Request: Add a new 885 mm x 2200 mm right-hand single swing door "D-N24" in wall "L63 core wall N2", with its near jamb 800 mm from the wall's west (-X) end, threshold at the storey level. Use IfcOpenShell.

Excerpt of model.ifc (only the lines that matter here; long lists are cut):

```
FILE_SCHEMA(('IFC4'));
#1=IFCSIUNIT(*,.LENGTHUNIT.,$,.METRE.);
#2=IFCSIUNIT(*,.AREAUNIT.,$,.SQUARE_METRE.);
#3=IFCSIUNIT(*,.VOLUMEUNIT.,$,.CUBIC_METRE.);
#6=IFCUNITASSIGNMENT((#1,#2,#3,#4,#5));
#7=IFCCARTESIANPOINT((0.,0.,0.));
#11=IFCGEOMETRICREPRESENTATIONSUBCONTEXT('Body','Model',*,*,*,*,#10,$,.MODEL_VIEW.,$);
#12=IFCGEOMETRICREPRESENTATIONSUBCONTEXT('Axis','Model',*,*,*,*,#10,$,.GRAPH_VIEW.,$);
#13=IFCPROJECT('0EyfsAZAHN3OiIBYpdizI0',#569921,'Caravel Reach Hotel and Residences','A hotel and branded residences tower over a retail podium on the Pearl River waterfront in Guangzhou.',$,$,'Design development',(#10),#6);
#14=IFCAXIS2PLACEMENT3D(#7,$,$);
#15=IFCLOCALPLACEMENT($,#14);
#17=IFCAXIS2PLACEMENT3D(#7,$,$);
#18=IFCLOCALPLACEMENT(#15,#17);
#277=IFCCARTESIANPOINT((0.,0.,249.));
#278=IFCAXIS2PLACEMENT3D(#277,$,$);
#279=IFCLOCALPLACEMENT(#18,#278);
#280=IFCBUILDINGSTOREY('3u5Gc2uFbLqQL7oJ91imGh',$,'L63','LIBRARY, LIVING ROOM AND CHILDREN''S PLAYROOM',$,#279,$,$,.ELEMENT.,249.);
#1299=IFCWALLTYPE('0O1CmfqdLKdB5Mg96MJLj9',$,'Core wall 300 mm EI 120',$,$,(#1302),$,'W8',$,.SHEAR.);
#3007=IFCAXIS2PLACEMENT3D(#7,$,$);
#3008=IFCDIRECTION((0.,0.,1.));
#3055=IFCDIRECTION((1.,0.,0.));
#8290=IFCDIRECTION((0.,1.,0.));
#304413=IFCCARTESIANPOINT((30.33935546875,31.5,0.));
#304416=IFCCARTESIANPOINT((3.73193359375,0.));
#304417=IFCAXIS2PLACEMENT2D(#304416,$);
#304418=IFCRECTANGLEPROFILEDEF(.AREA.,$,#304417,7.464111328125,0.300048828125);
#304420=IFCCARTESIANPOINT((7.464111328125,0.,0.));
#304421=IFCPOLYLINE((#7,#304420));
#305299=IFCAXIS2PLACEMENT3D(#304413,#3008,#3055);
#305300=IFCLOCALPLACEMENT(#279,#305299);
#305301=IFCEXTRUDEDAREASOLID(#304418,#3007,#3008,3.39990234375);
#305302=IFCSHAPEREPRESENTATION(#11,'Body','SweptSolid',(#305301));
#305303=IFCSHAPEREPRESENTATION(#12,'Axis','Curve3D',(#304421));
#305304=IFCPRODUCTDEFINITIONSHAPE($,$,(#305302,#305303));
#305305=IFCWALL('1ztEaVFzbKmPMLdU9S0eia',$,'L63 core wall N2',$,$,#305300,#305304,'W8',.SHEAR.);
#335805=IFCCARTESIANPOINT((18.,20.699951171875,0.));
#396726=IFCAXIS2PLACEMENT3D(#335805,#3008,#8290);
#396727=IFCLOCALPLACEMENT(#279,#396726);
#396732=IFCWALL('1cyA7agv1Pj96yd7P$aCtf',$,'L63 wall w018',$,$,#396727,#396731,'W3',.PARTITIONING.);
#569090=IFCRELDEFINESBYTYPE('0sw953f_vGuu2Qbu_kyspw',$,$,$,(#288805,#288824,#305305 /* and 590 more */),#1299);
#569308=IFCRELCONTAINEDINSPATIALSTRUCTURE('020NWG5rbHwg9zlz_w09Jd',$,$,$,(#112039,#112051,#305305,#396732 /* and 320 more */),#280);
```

```python
import numpy as np
import ifcopenshell
import ifcopenshell.api.feature
import ifcopenshell.api.geometry
import ifcopenshell.api.root
import ifcopenshell.api.spatial
import ifcopenshell.geom
import ifcopenshell.util.element
import ifcopenshell.util.placement
import ifcopenshell.util.representation
import ifcopenshell.util.shape
import ifcopenshell.util.unit

model = ifcopenshell.open("model.ifc")
unit_scale = ifcopenshell.util.unit.calculate_unit_scale(model)
settings = ifcopenshell.geom.settings()


def volume(element):
    """Net volume in cubic metres, openings subtracted."""
    shape = ifcopenshell.geom.create_shape(settings, element)
    return ifcopenshell.util.shape.get_volume(shape.geometry)


wall = model.by_guid("1ztEaVFzbKmPMLdU9S0eia")
storey = ifcopenshell.util.element.get_container(wall, ifc_class="IfcBuildingStorey")
context = ifcopenshell.util.representation.get_context(model, "Model", "Body", "MODEL_VIEW")
before = volume(wall)

width, height, from_end, sill = 0.885, 2.2, 0.8, 0.0  # metres

# The wall runs along its own X axis, and the end named is its -X end.
wall_shape = ifcopenshell.geom.create_shape(settings, wall)
x, y, z = ifcopenshell.util.shape.get_vertices(wall_shape.geometry).T
start = x.min() + from_end
face, thickness = float(y.min()), float(y.max() - y.min())
wall_matrix = ifcopenshell.util.placement.get_local_placement(wall.ObjectPlacement)
level = ifcopenshell.util.placement.get_local_placement(storey.ObjectPlacement)[2, 3]


def in_wall(x, y):
    """Placement at x, y metres in the wall's axes, at sill height."""
    matrix = wall_matrix.copy()
    matrix[:, 3] = wall_matrix @ np.array([x / unit_scale, y / unit_scale, 0.0, 1.0])
    matrix[2, 3] = level + sill / unit_scale
    return matrix


# Opening: a box that overshoots both wall faces by 50 mm.
opening = ifcopenshell.api.root.create_entity(model, ifc_class="IfcOpeningElement", predefined_type="OPENING")
box = ifcopenshell.api.geometry.add_wall_representation(
    model, context=context, length=width, height=height, thickness=thickness + 0.1
)
ifcopenshell.api.geometry.assign_representation(model, product=opening, representation=box)
ifcopenshell.api.geometry.edit_object_placement(model, product=opening, matrix=in_wall(start, face - 0.05), is_si=False)
ifcopenshell.api.feature.add_feature(model, feature=opening, element=wall)

door = ifcopenshell.api.root.create_entity(model, ifc_class="IfcDoor", name="D-N24", predefined_type="DOOR")
door.OverallWidth, door.OverallHeight = width / unit_scale, height / unit_scale
door.OperationType = "SINGLE_SWING_RIGHT"
body = ifcopenshell.api.geometry.add_door_representation(
    model,
    context=context,
    overall_width=door.OverallWidth,
    overall_height=door.OverallHeight,
    operation_type="SINGLE_SWING_RIGHT",
    lining_properties={"LiningDepth": thickness / unit_scale, "ThresholdDepth": thickness / unit_scale},
)
ifcopenshell.api.geometry.assign_representation(model, product=door, representation=body)
ifcopenshell.api.spatial.assign_container(model, products=[door], relating_structure=storey)
ifcopenshell.api.feature.add_filling(model, opening=opening, element=door)

# The lining spans the wall, so the door starts at the wall face.
ifcopenshell.api.geometry.edit_object_placement(model, product=door, matrix=in_wall(start, face), is_si=False)

after = volume(wall)

print(f"wall volume {before:.3f} -> {after:.3f} m3")

model.write("model_edited.ifc")
```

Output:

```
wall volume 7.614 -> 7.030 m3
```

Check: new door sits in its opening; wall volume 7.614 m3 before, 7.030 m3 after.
